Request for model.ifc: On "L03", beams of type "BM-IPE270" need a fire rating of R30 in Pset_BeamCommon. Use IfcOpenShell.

First a look at what the model holds.

```python
import ifcopenshell
import ifcopenshell.util.element

model = ifcopenshell.open("model.ifc")
print(model.schema)
storey = next(s for s in model.by_type("IfcBuildingStorey") if s.Name == "L03")
beams = [e for e in ifcopenshell.util.element.get_decomposition(storey) if e.is_a("IfcBeam")]
seen = {}
for e in beams:
    element_type = ifcopenshell.util.element.get_type(e)
    key = (element_type.Name if element_type != e and element_type else None, ifcopenshell.util.element.get_pset(e, "Pset_BeamCommon", "FireRating"))
    seen[key] = seen.get(key, 0) + 1
for (name, value), count in sorted(seen.items(), key=str):
    print(count, "x", name, "|", value)
```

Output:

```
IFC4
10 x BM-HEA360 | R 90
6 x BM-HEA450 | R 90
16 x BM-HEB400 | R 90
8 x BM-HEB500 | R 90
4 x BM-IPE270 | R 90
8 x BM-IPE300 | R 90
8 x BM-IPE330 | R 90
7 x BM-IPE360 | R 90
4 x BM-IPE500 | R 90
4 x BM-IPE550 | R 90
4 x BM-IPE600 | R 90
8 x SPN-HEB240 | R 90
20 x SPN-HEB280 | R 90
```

```python
import ifcopenshell
import ifcopenshell.api.pset
import ifcopenshell.util.element

model = ifcopenshell.open("model.ifc")

storey = next(s for s in model.by_type("IfcBuildingStorey") if s.Name == "L03")
beams = [e for e in ifcopenshell.util.element.get_decomposition(storey) if e.is_a("IfcBeam")]

count = 0
for e in beams:
    element_type = ifcopenshell.util.element.get_type(e)
    if element_type in (None, e) or element_type.Name != "BM-IPE270":
        continue
    # add_pset returns the element's existing set when there is one.
    pset = ifcopenshell.api.pset.add_pset(model, product=e, name="Pset_BeamCommon")
    ifcopenshell.api.pset.edit_pset(model, pset=pset, properties={"FireRating": "R30"})
    count += 1

print(count, "beams updated")

model.write("model_updated.ifc")
```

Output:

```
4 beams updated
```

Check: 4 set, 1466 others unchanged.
